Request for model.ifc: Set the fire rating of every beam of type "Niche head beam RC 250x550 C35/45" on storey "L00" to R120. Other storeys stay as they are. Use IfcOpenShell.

First a look at what the model holds.

```python
import ifcopenshell
import ifcopenshell.util.element

model = ifcopenshell.open("model.ifc")
print(model.schema)
storey = next(s for s in model.by_type("IfcBuildingStorey") if s.Name == "L00")
beams = [e for e in ifcopenshell.util.element.get_decomposition(storey) if e.is_a("IfcBeam")]
seen = {}
for e in beams:
    element_type = ifcopenshell.util.element.get_type(e)
    key = (element_type.Name if element_type != e and element_type else None, ifcopenshell.util.element.get_pset(e, "Pset_BeamCommon", "FireRating"))
    seen[key] = seen.get(key, 0) + 1
for (name, value), count in sorted(seen.items(), key=str):
    print(count, "x", name, "|", value)
```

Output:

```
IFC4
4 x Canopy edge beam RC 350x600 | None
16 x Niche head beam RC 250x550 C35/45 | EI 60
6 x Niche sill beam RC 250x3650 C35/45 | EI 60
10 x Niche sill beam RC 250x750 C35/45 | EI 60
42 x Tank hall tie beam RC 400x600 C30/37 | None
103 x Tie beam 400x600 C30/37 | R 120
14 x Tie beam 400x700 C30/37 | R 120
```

```python
import ifcopenshell
import ifcopenshell.api.pset
import ifcopenshell.util.element

model = ifcopenshell.open("model.ifc")

storey = next(s for s in model.by_type("IfcBuildingStorey") if s.Name == "L00")
beams = [e for e in ifcopenshell.util.element.get_decomposition(storey) if e.is_a("IfcBeam")]

count = 0
for e in beams:
    element_type = ifcopenshell.util.element.get_type(e)
    if element_type in (None, e) or element_type.Name != "Niche head beam RC 250x550 C35/45":
        continue
    # add_pset returns the element's existing set when there is one.
    pset = ifcopenshell.api.pset.add_pset(model, product=e, name="Pset_BeamCommon")
    ifcopenshell.api.pset.edit_pset(model, pset=pset, properties={"FireRating": "R120"})
    count += 1

print(count, "beams updated")

model.write("model_v2.ifc")
```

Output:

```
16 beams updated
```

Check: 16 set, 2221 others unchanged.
